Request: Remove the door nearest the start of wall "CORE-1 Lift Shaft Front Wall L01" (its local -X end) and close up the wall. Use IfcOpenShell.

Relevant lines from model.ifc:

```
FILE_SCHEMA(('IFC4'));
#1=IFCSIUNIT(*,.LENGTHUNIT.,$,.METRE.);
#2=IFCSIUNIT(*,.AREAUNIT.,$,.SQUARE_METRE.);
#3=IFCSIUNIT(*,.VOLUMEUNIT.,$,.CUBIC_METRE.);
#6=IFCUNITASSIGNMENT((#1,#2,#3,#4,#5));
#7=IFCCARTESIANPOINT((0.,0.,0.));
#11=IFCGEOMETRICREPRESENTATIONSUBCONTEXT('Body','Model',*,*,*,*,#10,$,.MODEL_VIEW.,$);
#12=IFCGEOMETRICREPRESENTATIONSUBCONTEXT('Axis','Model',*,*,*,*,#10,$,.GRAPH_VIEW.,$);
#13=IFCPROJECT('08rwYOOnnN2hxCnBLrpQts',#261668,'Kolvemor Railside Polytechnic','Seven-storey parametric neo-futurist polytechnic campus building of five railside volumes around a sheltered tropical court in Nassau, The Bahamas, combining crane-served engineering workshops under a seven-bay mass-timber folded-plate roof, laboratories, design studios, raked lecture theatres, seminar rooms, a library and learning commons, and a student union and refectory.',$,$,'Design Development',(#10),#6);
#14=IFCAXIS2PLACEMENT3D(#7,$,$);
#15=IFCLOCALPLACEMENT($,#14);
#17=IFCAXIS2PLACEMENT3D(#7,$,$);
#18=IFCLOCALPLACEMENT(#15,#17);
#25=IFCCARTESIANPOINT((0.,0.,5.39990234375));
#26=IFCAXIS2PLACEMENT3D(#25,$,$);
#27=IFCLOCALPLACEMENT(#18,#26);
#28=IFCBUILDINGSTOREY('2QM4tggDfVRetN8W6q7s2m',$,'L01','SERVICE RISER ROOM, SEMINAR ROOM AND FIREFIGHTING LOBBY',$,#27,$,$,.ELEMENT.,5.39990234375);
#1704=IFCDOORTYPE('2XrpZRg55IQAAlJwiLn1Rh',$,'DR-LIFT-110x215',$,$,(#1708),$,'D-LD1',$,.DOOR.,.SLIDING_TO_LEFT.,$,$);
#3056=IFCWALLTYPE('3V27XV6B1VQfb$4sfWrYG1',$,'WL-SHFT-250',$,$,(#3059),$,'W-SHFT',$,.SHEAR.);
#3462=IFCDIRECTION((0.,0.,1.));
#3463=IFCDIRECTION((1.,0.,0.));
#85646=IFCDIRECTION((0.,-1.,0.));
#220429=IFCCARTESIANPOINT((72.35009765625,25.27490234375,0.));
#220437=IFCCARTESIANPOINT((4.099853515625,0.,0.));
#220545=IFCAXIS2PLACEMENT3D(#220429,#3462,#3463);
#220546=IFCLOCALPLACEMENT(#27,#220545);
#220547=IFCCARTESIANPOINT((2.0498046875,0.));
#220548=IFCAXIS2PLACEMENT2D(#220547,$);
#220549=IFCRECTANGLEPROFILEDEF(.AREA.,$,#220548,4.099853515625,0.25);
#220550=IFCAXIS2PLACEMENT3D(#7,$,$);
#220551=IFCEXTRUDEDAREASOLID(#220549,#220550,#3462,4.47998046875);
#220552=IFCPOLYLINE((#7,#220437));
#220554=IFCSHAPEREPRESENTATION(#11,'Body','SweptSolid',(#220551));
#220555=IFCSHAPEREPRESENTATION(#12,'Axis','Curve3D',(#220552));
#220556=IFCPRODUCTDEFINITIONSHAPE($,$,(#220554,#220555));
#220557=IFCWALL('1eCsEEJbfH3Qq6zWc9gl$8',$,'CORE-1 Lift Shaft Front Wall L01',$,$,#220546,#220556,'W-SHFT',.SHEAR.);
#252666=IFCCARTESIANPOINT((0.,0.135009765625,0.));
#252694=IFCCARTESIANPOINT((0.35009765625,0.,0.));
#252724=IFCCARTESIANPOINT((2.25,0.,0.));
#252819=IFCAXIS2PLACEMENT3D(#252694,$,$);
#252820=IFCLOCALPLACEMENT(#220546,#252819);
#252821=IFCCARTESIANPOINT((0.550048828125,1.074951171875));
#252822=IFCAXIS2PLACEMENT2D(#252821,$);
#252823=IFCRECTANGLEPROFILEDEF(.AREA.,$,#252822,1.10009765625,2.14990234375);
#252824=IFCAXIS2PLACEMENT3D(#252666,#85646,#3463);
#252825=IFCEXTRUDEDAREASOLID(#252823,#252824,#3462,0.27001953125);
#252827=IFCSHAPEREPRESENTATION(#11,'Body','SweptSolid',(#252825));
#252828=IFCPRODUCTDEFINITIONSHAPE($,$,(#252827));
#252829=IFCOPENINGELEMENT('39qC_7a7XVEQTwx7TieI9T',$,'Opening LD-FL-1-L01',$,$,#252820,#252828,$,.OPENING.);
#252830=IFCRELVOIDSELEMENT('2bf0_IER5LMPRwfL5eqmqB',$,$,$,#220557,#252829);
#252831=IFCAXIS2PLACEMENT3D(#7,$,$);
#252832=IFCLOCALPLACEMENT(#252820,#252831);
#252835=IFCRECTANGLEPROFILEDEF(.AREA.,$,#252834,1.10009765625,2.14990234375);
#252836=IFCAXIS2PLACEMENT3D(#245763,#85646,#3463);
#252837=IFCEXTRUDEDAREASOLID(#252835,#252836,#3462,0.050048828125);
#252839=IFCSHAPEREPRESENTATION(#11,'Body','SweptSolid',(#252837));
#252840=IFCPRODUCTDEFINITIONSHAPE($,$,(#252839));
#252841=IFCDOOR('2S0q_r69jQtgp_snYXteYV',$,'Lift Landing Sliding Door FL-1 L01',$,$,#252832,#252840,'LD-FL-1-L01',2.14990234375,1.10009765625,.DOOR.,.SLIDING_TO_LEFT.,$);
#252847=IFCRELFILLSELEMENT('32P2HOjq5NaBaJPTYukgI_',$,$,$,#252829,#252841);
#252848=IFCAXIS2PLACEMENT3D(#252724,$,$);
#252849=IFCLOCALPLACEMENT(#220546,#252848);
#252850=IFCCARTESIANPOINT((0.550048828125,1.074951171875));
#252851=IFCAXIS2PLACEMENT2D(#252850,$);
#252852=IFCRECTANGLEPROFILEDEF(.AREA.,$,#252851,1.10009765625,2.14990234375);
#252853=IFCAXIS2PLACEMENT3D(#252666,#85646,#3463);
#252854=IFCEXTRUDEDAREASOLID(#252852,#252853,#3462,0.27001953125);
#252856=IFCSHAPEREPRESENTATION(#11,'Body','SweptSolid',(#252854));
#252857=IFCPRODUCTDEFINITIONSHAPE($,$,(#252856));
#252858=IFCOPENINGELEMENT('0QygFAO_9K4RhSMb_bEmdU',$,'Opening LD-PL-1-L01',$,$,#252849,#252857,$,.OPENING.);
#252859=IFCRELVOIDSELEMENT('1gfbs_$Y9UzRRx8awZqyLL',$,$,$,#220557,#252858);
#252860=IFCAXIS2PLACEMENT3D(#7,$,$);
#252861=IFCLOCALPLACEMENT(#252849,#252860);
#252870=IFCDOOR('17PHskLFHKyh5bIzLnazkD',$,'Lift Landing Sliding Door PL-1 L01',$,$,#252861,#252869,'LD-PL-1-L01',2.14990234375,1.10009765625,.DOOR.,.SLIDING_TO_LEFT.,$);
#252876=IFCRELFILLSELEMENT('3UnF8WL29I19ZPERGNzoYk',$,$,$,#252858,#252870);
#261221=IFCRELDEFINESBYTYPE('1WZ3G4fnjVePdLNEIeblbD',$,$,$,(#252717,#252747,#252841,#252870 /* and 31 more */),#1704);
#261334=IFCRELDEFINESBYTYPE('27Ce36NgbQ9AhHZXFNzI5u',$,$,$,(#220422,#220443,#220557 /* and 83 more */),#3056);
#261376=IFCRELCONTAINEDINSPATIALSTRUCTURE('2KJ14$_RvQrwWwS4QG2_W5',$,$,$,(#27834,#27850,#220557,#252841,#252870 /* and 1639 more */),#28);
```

```python
import ifcopenshell
import ifcopenshell.api.feature
import ifcopenshell.api.root
import ifcopenshell.geom
import ifcopenshell.util.shape

model = ifcopenshell.open("model.ifc")
settings = ifcopenshell.geom.settings()


def volume(element):
    """Net volume in cubic metres, openings subtracted."""
    shape = ifcopenshell.geom.create_shape(settings, element)
    return ifcopenshell.util.shape.get_volume(shape.geometry)


door = model.by_guid("2S0q_r69jQtgp_snYXteYV")
opening = door.FillsVoids[0].RelatingOpeningElement
wall = opening.VoidsElements[0].RelatingBuildingElement
before = volume(wall)

ifcopenshell.api.root.remove_product(model, product=door)
ifcopenshell.api.feature.remove_feature(model, feature=opening)

after = volume(wall)

print(f"wall volume {before:.3f} -> {after:.3f} m3")

model.write("model_updated.ifc")
```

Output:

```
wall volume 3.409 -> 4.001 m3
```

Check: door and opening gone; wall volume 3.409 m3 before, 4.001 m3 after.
